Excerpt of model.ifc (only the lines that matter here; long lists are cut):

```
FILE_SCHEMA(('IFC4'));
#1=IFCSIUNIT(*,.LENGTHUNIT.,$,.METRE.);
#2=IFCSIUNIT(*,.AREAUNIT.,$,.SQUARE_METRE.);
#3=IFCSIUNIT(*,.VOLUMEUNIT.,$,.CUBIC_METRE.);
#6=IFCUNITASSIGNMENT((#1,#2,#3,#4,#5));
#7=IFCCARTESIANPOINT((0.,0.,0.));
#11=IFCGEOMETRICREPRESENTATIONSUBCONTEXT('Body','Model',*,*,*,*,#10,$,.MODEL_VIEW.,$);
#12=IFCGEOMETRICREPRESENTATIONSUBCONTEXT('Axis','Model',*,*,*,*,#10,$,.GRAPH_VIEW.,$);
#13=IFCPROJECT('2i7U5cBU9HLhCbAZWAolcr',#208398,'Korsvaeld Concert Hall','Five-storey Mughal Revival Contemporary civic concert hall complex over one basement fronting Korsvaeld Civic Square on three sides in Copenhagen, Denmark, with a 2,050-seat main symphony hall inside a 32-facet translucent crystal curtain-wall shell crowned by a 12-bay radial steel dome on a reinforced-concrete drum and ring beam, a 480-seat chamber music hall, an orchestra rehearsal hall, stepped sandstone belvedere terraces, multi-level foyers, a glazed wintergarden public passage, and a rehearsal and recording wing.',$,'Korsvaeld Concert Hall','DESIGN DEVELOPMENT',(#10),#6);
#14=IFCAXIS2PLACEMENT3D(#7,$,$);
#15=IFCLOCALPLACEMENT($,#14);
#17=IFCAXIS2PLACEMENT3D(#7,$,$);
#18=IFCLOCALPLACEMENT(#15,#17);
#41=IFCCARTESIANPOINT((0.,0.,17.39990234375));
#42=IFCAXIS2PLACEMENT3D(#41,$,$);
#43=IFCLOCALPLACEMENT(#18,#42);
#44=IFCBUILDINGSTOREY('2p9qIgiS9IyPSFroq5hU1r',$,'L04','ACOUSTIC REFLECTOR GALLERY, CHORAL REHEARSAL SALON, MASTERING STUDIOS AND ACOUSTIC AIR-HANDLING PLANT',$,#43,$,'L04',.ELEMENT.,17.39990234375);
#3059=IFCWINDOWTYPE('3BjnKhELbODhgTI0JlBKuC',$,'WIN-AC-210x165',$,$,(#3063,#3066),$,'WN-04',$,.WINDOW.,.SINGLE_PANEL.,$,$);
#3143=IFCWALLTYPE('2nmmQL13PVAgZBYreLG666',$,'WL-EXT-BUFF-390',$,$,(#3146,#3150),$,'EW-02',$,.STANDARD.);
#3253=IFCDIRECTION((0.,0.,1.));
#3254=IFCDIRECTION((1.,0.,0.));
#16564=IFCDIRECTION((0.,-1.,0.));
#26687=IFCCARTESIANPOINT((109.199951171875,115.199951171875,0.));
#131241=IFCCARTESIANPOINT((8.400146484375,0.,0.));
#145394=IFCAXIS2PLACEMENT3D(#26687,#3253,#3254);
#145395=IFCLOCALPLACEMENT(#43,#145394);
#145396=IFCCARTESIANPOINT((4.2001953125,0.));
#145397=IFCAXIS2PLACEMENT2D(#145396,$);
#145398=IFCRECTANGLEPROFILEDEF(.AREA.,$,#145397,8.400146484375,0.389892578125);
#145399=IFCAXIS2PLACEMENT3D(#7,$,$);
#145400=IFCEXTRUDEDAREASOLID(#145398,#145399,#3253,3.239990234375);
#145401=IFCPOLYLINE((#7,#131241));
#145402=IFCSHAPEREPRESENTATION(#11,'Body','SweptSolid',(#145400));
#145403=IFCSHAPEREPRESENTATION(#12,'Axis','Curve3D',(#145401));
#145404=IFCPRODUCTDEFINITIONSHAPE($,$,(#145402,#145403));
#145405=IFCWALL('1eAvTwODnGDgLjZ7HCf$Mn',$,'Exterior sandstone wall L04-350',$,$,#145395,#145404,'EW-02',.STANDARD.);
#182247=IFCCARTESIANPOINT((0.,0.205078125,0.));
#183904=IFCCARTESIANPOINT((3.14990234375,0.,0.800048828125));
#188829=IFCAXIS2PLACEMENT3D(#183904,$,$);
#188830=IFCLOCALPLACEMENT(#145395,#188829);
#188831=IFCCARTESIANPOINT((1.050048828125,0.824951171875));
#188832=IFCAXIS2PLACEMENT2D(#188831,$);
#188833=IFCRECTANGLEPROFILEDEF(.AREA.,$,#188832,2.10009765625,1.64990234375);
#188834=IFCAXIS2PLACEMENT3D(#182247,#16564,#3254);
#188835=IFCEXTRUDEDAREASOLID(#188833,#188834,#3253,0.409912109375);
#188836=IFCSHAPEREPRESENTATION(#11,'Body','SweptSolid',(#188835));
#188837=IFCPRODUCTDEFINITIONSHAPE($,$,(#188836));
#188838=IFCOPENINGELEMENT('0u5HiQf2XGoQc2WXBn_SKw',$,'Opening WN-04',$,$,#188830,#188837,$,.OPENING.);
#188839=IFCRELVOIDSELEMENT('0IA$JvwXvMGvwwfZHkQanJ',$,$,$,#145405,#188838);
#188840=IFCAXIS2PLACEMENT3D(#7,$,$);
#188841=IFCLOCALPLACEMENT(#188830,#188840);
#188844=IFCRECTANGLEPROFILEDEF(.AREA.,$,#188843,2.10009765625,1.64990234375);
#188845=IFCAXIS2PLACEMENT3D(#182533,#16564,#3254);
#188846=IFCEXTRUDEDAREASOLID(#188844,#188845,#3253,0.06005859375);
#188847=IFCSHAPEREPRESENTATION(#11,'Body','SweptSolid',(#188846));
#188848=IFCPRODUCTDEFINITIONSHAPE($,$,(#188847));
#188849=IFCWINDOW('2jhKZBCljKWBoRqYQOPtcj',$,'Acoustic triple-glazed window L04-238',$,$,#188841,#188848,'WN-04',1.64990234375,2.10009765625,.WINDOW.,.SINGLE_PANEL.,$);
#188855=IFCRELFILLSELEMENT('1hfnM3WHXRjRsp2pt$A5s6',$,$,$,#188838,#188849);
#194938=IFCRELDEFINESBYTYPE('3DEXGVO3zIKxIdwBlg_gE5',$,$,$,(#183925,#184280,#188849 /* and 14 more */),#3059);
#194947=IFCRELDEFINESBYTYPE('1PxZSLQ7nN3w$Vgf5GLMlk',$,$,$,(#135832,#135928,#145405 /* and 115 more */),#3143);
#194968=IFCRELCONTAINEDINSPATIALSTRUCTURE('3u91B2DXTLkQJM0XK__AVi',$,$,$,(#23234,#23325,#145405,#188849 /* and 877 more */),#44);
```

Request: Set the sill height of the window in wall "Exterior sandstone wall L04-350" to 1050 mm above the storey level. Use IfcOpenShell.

```python
import numpy as np
import ifcopenshell
import ifcopenshell.api.geometry
import ifcopenshell.geom
import ifcopenshell.util.element
import ifcopenshell.util.placement
import ifcopenshell.util.shape
import ifcopenshell.util.unit

model = ifcopenshell.open("model.ifc")
unit_scale = ifcopenshell.util.unit.calculate_unit_scale(model)

window = model.by_id(188849)
opening = window.FillsVoids[0].RelatingOpeningElement
storey = ifcopenshell.util.element.get_container(window, ifc_class="IfcBuildingStorey")
level = ifcopenshell.util.placement.get_local_placement(storey.ObjectPlacement)[2, 3]

# The opening's origin need not be at the sill, so measure its lowest point.
shape = ifcopenshell.geom.create_shape(ifcopenshell.geom.settings(), opening)
bottom = ifcopenshell.util.shape.get_shape_bottom_elevation(shape, shape.geometry) / unit_scale
dz = level + 1.05 / unit_scale - bottom

shift = np.array([0.0, 0.0, dz])
# The window is placed relative to its opening, so it follows when the opening moves.
matrix = ifcopenshell.util.placement.get_local_placement(opening.ObjectPlacement)
matrix[:3, 3] += shift
ifcopenshell.api.geometry.edit_object_placement(
    model, product=opening, matrix=matrix, is_si=False, should_transform_children=True
)

print(f"moved by {dz * unit_scale:+.3f} m")

model.write("model-out.ifc")
```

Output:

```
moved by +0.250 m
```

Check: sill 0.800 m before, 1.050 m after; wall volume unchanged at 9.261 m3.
